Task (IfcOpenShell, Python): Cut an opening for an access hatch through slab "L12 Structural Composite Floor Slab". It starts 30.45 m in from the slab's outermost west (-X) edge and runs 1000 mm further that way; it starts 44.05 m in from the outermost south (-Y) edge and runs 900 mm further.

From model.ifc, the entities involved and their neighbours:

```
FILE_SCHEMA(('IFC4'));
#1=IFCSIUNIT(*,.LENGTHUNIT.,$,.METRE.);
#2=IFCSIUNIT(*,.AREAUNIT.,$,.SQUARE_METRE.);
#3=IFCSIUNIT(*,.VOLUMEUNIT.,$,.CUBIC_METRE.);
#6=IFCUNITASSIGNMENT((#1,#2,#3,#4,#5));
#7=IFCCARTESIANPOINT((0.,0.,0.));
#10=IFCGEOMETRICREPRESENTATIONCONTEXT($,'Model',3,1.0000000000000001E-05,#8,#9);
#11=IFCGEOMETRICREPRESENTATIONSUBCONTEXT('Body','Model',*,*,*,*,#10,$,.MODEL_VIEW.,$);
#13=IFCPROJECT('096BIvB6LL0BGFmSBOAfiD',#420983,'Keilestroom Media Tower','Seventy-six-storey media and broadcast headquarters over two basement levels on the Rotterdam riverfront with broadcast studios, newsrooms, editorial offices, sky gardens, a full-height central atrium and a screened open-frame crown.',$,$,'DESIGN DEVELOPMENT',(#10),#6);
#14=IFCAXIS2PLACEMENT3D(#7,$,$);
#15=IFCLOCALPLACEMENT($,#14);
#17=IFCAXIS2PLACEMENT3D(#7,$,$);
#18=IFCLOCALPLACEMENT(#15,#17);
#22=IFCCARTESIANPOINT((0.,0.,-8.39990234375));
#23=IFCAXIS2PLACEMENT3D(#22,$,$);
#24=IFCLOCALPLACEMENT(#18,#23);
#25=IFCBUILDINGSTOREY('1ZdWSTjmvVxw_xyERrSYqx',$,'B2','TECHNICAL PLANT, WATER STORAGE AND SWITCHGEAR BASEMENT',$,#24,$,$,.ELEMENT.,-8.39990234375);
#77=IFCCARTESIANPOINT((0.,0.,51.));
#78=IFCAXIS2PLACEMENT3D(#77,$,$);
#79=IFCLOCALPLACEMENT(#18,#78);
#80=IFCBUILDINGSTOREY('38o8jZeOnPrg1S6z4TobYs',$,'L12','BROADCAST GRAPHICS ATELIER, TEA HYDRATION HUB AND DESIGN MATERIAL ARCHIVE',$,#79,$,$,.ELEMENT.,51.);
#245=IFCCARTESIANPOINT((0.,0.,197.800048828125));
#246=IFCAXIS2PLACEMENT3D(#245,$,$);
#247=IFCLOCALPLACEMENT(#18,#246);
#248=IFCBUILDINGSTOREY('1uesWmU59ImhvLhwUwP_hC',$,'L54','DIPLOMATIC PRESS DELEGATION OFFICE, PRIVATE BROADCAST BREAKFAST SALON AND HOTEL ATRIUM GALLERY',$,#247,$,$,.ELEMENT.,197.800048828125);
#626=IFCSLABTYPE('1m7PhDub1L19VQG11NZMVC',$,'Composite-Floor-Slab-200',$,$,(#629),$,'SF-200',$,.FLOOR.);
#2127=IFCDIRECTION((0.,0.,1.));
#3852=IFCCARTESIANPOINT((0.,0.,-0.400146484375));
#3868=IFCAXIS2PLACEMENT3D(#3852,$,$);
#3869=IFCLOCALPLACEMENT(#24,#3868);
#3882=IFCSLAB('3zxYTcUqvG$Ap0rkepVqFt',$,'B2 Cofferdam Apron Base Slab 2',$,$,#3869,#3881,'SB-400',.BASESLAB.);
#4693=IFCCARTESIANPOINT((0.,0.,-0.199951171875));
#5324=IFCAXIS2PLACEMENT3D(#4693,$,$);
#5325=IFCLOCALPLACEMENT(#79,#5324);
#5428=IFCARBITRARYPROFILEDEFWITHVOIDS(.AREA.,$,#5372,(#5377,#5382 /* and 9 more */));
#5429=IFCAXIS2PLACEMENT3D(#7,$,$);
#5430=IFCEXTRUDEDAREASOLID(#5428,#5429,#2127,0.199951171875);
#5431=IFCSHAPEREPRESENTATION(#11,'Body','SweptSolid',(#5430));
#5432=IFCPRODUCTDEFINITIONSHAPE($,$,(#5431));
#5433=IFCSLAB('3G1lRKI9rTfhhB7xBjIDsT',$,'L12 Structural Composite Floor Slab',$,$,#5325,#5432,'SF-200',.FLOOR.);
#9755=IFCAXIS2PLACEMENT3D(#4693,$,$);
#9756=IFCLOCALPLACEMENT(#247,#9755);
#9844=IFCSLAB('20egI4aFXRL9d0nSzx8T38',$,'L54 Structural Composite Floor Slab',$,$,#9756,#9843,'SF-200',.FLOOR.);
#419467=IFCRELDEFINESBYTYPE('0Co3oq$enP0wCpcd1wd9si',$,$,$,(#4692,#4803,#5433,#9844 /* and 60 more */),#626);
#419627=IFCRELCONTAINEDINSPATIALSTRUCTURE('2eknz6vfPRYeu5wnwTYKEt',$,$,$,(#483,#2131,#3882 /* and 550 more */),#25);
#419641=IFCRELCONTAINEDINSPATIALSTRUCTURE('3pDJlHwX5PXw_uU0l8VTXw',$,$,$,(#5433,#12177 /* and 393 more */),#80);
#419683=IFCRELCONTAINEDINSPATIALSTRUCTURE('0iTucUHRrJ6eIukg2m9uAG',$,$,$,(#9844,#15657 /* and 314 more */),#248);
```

```python
import numpy as np
import ifcopenshell
import ifcopenshell.api.feature
import ifcopenshell.api.geometry
import ifcopenshell.api.root
import ifcopenshell.geom
import ifcopenshell.util.placement
import ifcopenshell.util.representation
import ifcopenshell.util.shape
import ifcopenshell.util.unit

model = ifcopenshell.open("model.ifc")
unit_scale = ifcopenshell.util.unit.calculate_unit_scale(model)
settings = ifcopenshell.geom.settings()


def volume(element):
    """Net volume in cubic metres, openings subtracted."""
    shape = ifcopenshell.geom.create_shape(settings, element)
    return ifcopenshell.util.shape.get_volume(shape.geometry)


slab = model.by_id(5433)
before = volume(slab)

# Extent in the slab's own axes, in metres. The edges named are its -X and -Y sides.
slab_shape = ifcopenshell.geom.create_shape(settings, slab)
vertices = ifcopenshell.util.shape.get_vertices(slab_shape.geometry)
x_min, y_min, bottom = vertices.min(axis=0)
top = vertices[:, 2].max()

opening = ifcopenshell.api.root.create_entity(model, ifc_class="IfcOpeningElement", name="Access hatch opening", predefined_type="OPENING")
context = ifcopenshell.util.representation.get_context(model, "Model", "Body", "MODEL_VIEW")
width, depth = 1, 0.9
outline = [(0.0, 0.0), (width, 0.0), (width, depth), (0.0, depth), (0.0, 0.0)]
# Overshoot both faces by 50 mm so the cut is clean.
shape = ifcopenshell.api.geometry.add_slab_representation(
    model, context=context, depth=top - bottom + 0.1, polyline=outline
)
ifcopenshell.api.geometry.assign_representation(model, product=opening, representation=shape)

matrix = ifcopenshell.util.placement.get_local_placement(slab.ObjectPlacement)
matrix[:, 3] = matrix @ np.append(np.array([x_min + 30.45, y_min + 44.05, bottom - 0.05]) / unit_scale, 1.0)
ifcopenshell.api.geometry.edit_object_placement(model, product=opening, matrix=matrix, is_si=False)
ifcopenshell.api.feature.add_feature(model, feature=opening, element=slab)

after = volume(slab)

print(f"slab volume {before:.3f} -> {after:.3f} m3")

model.write("model-out.ifc")
```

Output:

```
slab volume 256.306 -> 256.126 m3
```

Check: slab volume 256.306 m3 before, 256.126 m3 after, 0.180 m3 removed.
